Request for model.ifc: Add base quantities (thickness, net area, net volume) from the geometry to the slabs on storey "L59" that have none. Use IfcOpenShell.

First a look at what the model holds.

```python
import ifcopenshell
import ifcopenshell.util.element
import ifcopenshell.util.unit

model = ifcopenshell.open("model.ifc")
print(model.schema)
for unit_type in ("LENGTHUNIT", "AREAUNIT", "VOLUMEUNIT"):
    print(unit_type, ifcopenshell.util.unit.calculate_unit_scale(model, unit_type))
storey = next(s for s in model.by_type("IfcBuildingStorey") if s.Name == "L59")
slabs = [e for e in ifcopenshell.util.element.get_decomposition(storey) if e.is_a("IfcSlab")]
for e in sorted(slabs, key=lambda e: e.id()):
    print(e.id(), e.is_a(), e.Name, list(ifcopenshell.util.element.get_psets(e, qtos_only=True)), sep=" | ")
```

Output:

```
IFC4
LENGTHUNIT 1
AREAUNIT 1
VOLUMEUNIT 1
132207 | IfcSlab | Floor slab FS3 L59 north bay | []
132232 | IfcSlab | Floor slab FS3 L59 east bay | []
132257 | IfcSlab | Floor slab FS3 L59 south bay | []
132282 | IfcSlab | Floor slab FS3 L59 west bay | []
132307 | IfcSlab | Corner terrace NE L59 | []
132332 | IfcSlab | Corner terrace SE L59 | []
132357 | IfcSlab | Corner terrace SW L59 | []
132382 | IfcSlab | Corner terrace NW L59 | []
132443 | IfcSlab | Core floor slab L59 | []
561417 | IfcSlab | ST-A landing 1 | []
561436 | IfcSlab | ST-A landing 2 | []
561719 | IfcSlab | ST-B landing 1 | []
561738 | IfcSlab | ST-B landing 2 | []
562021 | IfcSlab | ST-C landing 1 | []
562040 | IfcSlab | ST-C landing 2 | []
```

```python
import ifcopenshell
import ifcopenshell.api.pset
import ifcopenshell.geom
import ifcopenshell.util.element
import ifcopenshell.util.shape
import ifcopenshell.util.unit

model = ifcopenshell.open("model.ifc")
unit_scale = ifcopenshell.util.unit.calculate_unit_scale(model)
area_scale = ifcopenshell.util.unit.calculate_unit_scale(model, "AREAUNIT")
volume_scale = ifcopenshell.util.unit.calculate_unit_scale(model, "VOLUMEUNIT")
settings = ifcopenshell.geom.settings()

storey = next(s for s in model.by_type("IfcBuildingStorey") if s.Name == "L59")
slabs = [e for e in ifcopenshell.util.element.get_decomposition(storey) if e.is_a("IfcSlab")]

for e in sorted(slabs, key=lambda e: e.id()):
    if ifcopenshell.util.element.get_psets(e, qtos_only=True, should_inherit=False):
        continue
    # Geometry comes back in metres, in the element's own axes.
    shape = ifcopenshell.geom.create_shape(settings, e)
    values = {
        "Width": ifcopenshell.util.shape.get_z(shape.geometry) / unit_scale,
        "NetArea": ifcopenshell.util.shape.get_footprint_area(shape.geometry) / area_scale,
        "NetVolume": ifcopenshell.util.shape.get_volume(shape.geometry) / volume_scale,
    }
    qto = ifcopenshell.api.pset.add_qto(model, product=e, name="Qto_SlabBaseQuantities")
    ifcopenshell.api.pset.edit_qto(model, qto=qto, properties=values)
    print(e.id(), {k: round(v, 3) for k, v in values.items()})

model.write("model_v2.ifc")
```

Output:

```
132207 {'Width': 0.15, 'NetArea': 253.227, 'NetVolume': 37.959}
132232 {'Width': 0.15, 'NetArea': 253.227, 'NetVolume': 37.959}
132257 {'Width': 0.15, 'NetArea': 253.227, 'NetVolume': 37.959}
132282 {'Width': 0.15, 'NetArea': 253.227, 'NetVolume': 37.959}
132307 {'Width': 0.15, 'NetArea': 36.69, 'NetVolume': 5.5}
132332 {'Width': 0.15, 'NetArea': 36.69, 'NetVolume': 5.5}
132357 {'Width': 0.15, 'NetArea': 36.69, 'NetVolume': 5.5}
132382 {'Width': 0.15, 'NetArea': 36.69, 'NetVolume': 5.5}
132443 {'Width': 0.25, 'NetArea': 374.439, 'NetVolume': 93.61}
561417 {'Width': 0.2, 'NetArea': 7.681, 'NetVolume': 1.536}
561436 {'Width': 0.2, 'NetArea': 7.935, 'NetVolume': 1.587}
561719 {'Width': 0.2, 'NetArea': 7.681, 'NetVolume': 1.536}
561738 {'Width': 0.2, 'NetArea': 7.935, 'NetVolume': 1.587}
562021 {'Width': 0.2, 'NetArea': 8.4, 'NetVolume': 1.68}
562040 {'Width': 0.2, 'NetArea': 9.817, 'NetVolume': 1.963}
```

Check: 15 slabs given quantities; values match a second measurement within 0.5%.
